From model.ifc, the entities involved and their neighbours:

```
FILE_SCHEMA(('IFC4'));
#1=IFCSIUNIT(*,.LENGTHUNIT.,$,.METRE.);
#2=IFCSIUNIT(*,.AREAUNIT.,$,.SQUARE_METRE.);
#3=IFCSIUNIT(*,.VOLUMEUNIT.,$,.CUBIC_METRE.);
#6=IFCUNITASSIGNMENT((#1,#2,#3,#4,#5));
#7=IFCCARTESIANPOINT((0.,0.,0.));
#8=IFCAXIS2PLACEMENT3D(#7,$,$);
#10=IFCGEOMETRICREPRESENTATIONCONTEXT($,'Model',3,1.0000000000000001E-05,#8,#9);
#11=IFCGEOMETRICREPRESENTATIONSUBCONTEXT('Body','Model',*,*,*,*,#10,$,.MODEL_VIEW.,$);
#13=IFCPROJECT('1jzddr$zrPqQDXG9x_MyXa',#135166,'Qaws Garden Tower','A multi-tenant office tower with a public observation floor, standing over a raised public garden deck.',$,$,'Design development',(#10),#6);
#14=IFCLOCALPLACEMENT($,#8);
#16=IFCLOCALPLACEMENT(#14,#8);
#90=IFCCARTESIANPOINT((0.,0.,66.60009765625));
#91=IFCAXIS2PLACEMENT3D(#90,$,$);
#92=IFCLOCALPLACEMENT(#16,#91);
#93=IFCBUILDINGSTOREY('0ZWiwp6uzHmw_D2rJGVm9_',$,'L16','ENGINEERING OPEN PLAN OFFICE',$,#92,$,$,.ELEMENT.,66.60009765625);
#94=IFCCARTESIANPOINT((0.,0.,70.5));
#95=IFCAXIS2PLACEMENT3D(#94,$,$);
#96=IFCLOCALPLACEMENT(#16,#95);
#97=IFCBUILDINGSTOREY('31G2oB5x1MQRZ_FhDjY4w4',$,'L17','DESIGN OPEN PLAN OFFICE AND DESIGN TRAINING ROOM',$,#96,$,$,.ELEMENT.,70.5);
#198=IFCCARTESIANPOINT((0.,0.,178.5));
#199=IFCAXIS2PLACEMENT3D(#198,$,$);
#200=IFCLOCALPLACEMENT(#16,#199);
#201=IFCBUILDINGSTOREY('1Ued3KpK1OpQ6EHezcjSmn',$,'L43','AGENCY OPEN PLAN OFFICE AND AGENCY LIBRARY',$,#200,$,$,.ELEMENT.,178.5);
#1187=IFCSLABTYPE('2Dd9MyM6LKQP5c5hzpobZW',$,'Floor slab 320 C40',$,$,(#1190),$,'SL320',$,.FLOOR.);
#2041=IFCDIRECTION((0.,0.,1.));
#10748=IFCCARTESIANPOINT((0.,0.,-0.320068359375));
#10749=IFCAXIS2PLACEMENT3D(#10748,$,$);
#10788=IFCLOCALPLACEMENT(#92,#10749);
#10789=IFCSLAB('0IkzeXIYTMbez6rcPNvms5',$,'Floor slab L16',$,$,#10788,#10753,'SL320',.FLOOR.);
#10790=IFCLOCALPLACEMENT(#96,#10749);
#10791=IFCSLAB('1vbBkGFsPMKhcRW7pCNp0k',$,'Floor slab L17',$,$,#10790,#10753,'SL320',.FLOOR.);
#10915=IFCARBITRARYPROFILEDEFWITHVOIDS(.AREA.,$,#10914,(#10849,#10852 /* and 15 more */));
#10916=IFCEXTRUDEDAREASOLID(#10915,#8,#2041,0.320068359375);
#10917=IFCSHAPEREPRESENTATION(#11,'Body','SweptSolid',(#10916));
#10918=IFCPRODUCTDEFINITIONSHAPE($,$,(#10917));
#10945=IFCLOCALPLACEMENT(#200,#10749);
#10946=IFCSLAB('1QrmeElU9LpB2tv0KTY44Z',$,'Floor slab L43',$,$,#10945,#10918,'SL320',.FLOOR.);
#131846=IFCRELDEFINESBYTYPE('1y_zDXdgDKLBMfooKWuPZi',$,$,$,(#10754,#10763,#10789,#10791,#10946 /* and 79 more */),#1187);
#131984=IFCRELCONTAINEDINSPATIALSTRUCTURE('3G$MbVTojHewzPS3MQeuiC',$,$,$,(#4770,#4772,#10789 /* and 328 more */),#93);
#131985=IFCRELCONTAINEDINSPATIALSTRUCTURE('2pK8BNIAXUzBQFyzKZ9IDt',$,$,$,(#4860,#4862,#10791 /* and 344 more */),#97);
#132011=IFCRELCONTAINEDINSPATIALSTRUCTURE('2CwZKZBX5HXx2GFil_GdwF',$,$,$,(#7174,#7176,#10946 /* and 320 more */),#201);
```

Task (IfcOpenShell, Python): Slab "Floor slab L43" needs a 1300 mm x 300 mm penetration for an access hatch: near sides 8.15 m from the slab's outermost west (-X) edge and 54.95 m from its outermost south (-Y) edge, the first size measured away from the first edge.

```python
import numpy as np
import ifcopenshell
import ifcopenshell.api.feature
import ifcopenshell.api.geometry
import ifcopenshell.api.root
import ifcopenshell.geom
import ifcopenshell.util.placement
import ifcopenshell.util.representation
import ifcopenshell.util.shape
import ifcopenshell.util.unit

model = ifcopenshell.open("model.ifc")
unit_scale = ifcopenshell.util.unit.calculate_unit_scale(model)
settings = ifcopenshell.geom.settings()


def volume(element):
    """Net volume in cubic metres, openings subtracted."""
    shape = ifcopenshell.geom.create_shape(settings, element)
    return ifcopenshell.util.shape.get_volume(shape.geometry)


slab = model.by_guid("1QrmeElU9LpB2tv0KTY44Z")
before = volume(slab)

# Extent in the slab's own axes, in metres. The edges named are its -X and -Y sides.
slab_shape = ifcopenshell.geom.create_shape(settings, slab)
vertices = ifcopenshell.util.shape.get_vertices(slab_shape.geometry)
x_min, y_min, bottom = vertices.min(axis=0)
top = vertices[:, 2].max()

opening = ifcopenshell.api.root.create_entity(model, ifc_class="IfcOpeningElement", name="Access hatch opening", predefined_type="OPENING")
context = ifcopenshell.util.representation.get_context(model, "Model", "Body", "MODEL_VIEW")
width, depth = 1.3, 0.3
outline = [(0.0, 0.0), (width, 0.0), (width, depth), (0.0, depth), (0.0, 0.0)]
# Overshoot both faces by 50 mm so the cut is clean.
shape = ifcopenshell.api.geometry.add_slab_representation(
    model, context=context, depth=top - bottom + 0.1, polyline=outline
)
ifcopenshell.api.geometry.assign_representation(model, product=opening, representation=shape)

matrix = ifcopenshell.util.placement.get_local_placement(slab.ObjectPlacement)
matrix[:, 3] = matrix @ np.append(np.array([x_min + 8.15, y_min + 54.95, bottom - 0.05]) / unit_scale, 1.0)
ifcopenshell.api.geometry.edit_object_placement(model, product=opening, matrix=matrix, is_si=False)
ifcopenshell.api.feature.add_feature(model, feature=opening, element=slab)

after = volume(slab)

print(f"slab volume {before:.3f} -> {after:.3f} m3")

model.write("model_edited.ifc")
```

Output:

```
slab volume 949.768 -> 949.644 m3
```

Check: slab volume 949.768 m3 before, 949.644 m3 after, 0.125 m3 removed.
